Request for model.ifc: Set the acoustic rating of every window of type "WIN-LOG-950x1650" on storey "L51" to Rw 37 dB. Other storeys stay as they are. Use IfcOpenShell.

First a look at what the model holds.

```python
import ifcopenshell
import ifcopenshell.util.element

model = ifcopenshell.open("model.ifc")
print(model.schema)
storey = next(s for s in model.by_type("IfcBuildingStorey") if s.Name == "L51")
windows = [e for e in ifcopenshell.util.element.get_decomposition(storey) if e.is_a("IfcWindow")]
seen = {}
for e in windows:
    element_type = ifcopenshell.util.element.get_type(e)
    key = (element_type.Name if element_type != e and element_type else None, ifcopenshell.util.element.get_pset(e, "Pset_WindowCommon", "AcousticRating"))
    seen[key] = seen.get(key, 0) + 1
for (name, value), count in sorted(seen.items(), key=str):
    print(count, "x", name, "|", value)
```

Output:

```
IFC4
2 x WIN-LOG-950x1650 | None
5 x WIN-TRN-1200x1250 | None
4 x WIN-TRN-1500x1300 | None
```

```python
import ifcopenshell
import ifcopenshell.api.pset
import ifcopenshell.util.element

model = ifcopenshell.open("model.ifc")

storey = next(s for s in model.by_type("IfcBuildingStorey") if s.Name == "L51")
windows = [e for e in ifcopenshell.util.element.get_decomposition(storey) if e.is_a("IfcWindow")]

count = 0
for e in windows:
    element_type = ifcopenshell.util.element.get_type(e)
    if element_type in (None, e) or element_type.Name != "WIN-LOG-950x1650":
        continue
    # add_pset returns the element's existing set when there is one.
    pset = ifcopenshell.api.pset.add_pset(model, product=e, name="Pset_WindowCommon")
    ifcopenshell.api.pset.edit_pset(model, pset=pset, properties={"AcousticRating": "Rw 37 dB"})
    count += 1

print(count, "windows updated")

model.write("model_updated.ifc")
```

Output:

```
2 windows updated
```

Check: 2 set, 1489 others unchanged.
